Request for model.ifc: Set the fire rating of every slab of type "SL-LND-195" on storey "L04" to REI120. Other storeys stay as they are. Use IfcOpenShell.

First a look at what the model holds.

```python
import ifcopenshell
import ifcopenshell.util.element

model = ifcopenshell.open("model.ifc")
print(model.schema)
storey = next(s for s in model.by_type("IfcBuildingStorey") if s.Name == "L04")
slabs = [e for e in ifcopenshell.util.element.get_decomposition(storey) if e.is_a("IfcSlab")]
seen = {}
for e in slabs:
    element_type = ifcopenshell.util.element.get_type(e)
    key = (element_type.Name if element_type != e and element_type else None, ifcopenshell.util.element.get_pset(e, "Pset_SlabCommon", "FireRating"))
    seen[key] = seen.get(key, 0) + 1
for (name, value), count in sorted(seen.items(), key=str):
    print(count, "x", name, "|", value)
```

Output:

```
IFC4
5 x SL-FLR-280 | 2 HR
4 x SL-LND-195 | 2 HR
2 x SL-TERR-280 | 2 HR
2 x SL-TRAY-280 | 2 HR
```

```python
import ifcopenshell
import ifcopenshell.api.pset
import ifcopenshell.util.element

model = ifcopenshell.open("model.ifc")

storey = next(s for s in model.by_type("IfcBuildingStorey") if s.Name == "L04")
slabs = [e for e in ifcopenshell.util.element.get_decomposition(storey) if e.is_a("IfcSlab")]

count = 0
for e in slabs:
    element_type = ifcopenshell.util.element.get_type(e)
    if element_type in (None, e) or element_type.Name != "SL-LND-195":
        continue
    # add_pset returns the element's existing set when there is one.
    pset = ifcopenshell.api.pset.add_pset(model, product=e, name="Pset_SlabCommon")
    ifcopenshell.api.pset.edit_pset(model, pset=pset, properties={"FireRating": "REI120"})
    count += 1

print(count, "slabs updated")

model.write("model_rev.ifc")
```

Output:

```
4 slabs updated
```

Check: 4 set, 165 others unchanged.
